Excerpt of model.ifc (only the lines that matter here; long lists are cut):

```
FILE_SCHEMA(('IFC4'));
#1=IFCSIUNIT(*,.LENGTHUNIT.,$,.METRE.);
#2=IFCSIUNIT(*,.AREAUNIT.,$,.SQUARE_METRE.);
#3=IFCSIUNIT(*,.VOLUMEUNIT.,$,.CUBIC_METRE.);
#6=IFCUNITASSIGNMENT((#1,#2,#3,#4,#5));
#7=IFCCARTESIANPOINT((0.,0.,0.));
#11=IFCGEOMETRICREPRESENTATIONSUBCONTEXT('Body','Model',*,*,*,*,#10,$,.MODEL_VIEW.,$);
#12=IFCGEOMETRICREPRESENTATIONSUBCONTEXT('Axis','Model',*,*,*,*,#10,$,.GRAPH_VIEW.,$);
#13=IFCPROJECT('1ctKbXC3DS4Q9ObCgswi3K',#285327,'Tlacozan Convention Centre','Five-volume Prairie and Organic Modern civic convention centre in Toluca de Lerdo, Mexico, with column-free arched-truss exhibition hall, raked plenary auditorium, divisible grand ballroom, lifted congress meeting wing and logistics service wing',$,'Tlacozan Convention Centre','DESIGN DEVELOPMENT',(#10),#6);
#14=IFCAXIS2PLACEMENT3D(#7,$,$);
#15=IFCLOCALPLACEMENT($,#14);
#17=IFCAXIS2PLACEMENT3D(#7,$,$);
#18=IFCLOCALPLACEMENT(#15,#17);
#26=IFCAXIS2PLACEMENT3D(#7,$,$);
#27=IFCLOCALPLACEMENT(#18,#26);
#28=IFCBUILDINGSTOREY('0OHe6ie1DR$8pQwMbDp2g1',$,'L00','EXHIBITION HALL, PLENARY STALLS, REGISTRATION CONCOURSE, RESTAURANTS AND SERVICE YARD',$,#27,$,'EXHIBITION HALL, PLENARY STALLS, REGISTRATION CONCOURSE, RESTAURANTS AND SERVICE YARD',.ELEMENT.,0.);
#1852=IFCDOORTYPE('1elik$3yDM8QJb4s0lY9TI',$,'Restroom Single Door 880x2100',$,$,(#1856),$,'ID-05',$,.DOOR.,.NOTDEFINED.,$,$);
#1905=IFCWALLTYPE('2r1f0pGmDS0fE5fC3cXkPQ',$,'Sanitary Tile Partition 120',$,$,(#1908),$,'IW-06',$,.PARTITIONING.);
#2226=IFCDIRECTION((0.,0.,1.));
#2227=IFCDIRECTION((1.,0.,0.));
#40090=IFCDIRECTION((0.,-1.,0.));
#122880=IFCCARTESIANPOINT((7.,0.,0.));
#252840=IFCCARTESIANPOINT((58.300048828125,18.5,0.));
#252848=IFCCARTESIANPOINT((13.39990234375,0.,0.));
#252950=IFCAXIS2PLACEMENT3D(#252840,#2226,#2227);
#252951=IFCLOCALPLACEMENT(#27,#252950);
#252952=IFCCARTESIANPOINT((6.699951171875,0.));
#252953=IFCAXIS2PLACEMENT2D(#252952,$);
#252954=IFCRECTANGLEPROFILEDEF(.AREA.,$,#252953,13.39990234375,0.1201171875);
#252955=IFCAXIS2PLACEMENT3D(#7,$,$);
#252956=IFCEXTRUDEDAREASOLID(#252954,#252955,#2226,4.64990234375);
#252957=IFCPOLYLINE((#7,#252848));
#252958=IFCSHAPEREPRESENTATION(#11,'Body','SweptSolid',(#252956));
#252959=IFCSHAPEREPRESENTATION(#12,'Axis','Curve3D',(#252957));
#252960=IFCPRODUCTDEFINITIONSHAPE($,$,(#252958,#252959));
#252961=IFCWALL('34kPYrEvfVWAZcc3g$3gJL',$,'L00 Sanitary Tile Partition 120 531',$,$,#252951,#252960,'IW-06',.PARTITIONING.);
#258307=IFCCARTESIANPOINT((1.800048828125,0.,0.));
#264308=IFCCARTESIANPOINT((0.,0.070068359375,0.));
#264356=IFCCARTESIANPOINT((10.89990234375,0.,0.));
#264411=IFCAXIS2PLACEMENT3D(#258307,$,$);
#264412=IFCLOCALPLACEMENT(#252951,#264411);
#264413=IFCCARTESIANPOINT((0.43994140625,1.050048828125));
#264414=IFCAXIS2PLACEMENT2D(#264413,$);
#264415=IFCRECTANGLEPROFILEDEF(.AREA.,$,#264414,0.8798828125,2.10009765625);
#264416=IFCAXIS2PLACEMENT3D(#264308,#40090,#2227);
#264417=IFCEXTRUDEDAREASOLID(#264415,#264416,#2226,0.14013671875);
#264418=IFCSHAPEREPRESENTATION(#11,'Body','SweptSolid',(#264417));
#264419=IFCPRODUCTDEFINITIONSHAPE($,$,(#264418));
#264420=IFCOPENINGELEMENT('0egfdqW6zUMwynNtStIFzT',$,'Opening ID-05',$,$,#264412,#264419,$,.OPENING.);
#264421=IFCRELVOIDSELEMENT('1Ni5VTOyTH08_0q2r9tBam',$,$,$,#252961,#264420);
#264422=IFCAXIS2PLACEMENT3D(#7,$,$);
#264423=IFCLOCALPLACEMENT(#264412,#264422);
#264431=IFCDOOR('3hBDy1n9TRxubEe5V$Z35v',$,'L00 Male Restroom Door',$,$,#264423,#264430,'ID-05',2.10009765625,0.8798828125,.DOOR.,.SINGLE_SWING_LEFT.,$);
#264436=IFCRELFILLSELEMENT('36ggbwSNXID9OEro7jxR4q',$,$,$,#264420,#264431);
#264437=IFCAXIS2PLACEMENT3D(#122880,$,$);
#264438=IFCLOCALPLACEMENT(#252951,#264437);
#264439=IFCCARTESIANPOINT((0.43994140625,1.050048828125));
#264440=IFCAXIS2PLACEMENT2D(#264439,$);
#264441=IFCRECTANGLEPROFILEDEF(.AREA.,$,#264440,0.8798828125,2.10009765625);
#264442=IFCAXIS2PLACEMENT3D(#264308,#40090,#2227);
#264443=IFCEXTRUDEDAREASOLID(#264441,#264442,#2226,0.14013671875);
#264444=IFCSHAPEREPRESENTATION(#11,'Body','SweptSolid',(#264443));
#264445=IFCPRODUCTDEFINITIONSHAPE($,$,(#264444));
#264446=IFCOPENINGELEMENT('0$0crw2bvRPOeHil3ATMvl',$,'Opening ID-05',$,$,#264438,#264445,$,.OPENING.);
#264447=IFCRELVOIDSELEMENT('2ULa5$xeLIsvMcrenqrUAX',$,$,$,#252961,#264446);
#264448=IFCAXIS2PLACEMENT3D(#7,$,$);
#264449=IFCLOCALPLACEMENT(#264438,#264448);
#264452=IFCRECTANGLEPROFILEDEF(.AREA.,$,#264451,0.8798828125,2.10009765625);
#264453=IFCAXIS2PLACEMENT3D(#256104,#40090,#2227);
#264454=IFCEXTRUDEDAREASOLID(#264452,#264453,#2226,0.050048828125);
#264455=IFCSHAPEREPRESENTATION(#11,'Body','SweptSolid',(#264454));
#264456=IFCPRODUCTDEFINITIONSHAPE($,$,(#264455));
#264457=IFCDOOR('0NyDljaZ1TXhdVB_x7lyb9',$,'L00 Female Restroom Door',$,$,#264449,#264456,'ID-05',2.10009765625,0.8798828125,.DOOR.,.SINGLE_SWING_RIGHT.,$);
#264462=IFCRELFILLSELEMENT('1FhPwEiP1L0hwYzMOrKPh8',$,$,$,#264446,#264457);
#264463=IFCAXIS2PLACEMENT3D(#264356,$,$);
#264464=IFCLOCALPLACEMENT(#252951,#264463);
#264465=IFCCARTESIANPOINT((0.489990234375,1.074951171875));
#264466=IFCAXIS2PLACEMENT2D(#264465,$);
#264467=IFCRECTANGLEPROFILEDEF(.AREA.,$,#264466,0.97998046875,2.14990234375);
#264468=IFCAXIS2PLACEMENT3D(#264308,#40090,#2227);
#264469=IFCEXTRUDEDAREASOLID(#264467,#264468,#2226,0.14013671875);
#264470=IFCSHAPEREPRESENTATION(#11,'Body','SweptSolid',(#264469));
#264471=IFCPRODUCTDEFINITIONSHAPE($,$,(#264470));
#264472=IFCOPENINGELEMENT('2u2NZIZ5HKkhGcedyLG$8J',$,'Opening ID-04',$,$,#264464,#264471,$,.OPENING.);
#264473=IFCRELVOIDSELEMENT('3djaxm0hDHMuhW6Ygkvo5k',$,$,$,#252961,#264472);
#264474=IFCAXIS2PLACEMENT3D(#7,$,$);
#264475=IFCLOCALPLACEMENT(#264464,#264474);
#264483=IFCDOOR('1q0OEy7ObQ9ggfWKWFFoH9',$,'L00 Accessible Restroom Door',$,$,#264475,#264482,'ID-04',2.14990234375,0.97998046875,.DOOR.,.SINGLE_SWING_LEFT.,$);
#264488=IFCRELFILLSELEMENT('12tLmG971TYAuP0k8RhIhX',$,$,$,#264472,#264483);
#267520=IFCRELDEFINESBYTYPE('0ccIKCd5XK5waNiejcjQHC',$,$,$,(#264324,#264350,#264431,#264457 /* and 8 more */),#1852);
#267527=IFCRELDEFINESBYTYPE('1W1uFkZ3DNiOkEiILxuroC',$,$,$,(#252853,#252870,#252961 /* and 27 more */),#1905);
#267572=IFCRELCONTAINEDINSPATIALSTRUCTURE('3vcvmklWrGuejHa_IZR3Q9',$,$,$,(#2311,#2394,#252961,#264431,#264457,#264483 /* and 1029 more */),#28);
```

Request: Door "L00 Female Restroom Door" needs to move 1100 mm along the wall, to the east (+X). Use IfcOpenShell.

```python
import ifcopenshell
import ifcopenshell.api.geometry
import ifcopenshell.util.placement

model = ifcopenshell.open("model.ifc")

door = model.by_guid("0NyDljaZ1TXhdVB_x7lyb9")
opening = door.FillsVoids[0].RelatingOpeningElement
wall = opening.VoidsElements[0].RelatingBuildingElement

wall_matrix = ifcopenshell.util.placement.get_local_placement(wall.ObjectPlacement)
shift = wall_matrix[:3, 0] * 1.1
before = ifcopenshell.util.placement.get_local_placement(door.ObjectPlacement)[:3, 3].copy()

# The door is placed relative to its opening, so it follows when the opening moves.
matrix = ifcopenshell.util.placement.get_local_placement(opening.ObjectPlacement)
matrix[:3, 3] += shift
ifcopenshell.api.geometry.edit_object_placement(
    model, product=opening, matrix=matrix, is_si=False, should_transform_children=True
)

after = ifcopenshell.util.placement.get_local_placement(door.ObjectPlacement)[:3, 3]
print("door moved by", (after - before).round(3) + 0.0)

model.write("model_edited.ifc")
```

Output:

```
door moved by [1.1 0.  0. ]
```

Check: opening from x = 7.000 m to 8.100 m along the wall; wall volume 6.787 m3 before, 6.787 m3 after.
